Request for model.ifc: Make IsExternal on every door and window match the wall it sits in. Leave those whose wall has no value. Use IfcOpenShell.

First a look at what the model holds.

```python
import ifcopenshell
import ifcopenshell.util.element

model = ifcopenshell.open("model.ifc")
print(model.schema)
seen = {}
for e in model.by_type("IfcDoor") + model.by_type("IfcWindow"):
    if not e.FillsVoids:
        continue
    host = e.FillsVoids[0].RelatingOpeningElement.VoidsElements[0].RelatingBuildingElement
    own = ifcopenshell.util.element.get_pset(e, f"Pset_{e.is_a()[3:].removesuffix('StandardCase')}Common", "IsExternal")
    wall = ifcopenshell.util.element.get_pset(host, "Pset_WallCommon", "IsExternal")
    seen[e.is_a(), own, wall] = seen.get((e.is_a(), own, wall), 0) + 1
for (cls, own, wall), count in sorted(seen.items(), key=str):
    print(count, cls, "IsExternal:", own, "| host wall:", wall)
```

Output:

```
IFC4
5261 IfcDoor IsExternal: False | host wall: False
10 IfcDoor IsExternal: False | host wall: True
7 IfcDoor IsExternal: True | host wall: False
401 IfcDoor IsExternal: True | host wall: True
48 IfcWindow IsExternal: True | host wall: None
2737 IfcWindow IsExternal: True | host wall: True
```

```python
import ifcopenshell
import ifcopenshell.api.pset
import ifcopenshell.util.element

model = ifcopenshell.open("model.ifc")

count = 0
for ifc_class, pset_name in (("IfcDoor", "Pset_DoorCommon"), ("IfcWindow", "Pset_WindowCommon")):
    for e in model.by_type(ifc_class):
        if not e.FillsVoids:
            continue
        host = e.FillsVoids[0].RelatingOpeningElement.VoidsElements[0].RelatingBuildingElement
        external = ifcopenshell.util.element.get_pset(host, "Pset_WallCommon", "IsExternal")
        if external is None or ifcopenshell.util.element.get_pset(e, pset_name, "IsExternal") == external:
            continue
        pset = ifcopenshell.api.pset.add_pset(model, product=e, name=pset_name)
        ifcopenshell.api.pset.edit_pset(model, pset=pset, properties={"IsExternal": external})
        count += 1

print(count, "updated")

model.write("model_rev.ifc")
```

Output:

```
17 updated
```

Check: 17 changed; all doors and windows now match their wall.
